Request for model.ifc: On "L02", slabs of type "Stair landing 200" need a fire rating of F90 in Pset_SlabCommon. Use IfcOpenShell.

First a look at what the model holds.

```python
import ifcopenshell
import ifcopenshell.util.element

model = ifcopenshell.open("model.ifc")
print(model.schema)
storey = next(s for s in model.by_type("IfcBuildingStorey") if s.Name == "L02")
slabs = [e for e in ifcopenshell.util.element.get_decomposition(storey) if e.is_a("IfcSlab")]
seen = {}
for e in slabs:
    element_type = ifcopenshell.util.element.get_type(e)
    key = (element_type.Name if element_type != e and element_type else None, ifcopenshell.util.element.get_pset(e, "Pset_SlabCommon", "FireRating"))
    seen[key] = seen.get(key, 0) + 1
for (name, value), count in sorted(seen.items(), key=str):
    print(count, "x", name, "|", value)
```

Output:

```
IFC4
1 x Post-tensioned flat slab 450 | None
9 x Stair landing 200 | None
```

```python
import ifcopenshell
import ifcopenshell.api.pset
import ifcopenshell.util.element

model = ifcopenshell.open("model.ifc")

storey = next(s for s in model.by_type("IfcBuildingStorey") if s.Name == "L02")
slabs = [e for e in ifcopenshell.util.element.get_decomposition(storey) if e.is_a("IfcSlab")]

count = 0
for e in slabs:
    element_type = ifcopenshell.util.element.get_type(e)
    if element_type in (None, e) or element_type.Name != "Stair landing 200":
        continue
    found = ifcopenshell.util.element.get_pset(e, "Pset_SlabCommon", should_inherit=False)
    if found:
        pset = model.by_id(found["id"])
        if len(ifcopenshell.util.element.get_elements_by_pset(pset)) > 1:
            pset = ifcopenshell.api.pset.unshare_pset(model, products=[e], pset=pset)[0]
    else:
        pset = ifcopenshell.api.pset.add_pset(model, product=e, name="Pset_SlabCommon")
    ifcopenshell.api.pset.edit_pset(model, pset=pset, properties={"FireRating": "F90"})
    count += 1

print(count, "slabs updated")

model.write("model_v2.ifc")
```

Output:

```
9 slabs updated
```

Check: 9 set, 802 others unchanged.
